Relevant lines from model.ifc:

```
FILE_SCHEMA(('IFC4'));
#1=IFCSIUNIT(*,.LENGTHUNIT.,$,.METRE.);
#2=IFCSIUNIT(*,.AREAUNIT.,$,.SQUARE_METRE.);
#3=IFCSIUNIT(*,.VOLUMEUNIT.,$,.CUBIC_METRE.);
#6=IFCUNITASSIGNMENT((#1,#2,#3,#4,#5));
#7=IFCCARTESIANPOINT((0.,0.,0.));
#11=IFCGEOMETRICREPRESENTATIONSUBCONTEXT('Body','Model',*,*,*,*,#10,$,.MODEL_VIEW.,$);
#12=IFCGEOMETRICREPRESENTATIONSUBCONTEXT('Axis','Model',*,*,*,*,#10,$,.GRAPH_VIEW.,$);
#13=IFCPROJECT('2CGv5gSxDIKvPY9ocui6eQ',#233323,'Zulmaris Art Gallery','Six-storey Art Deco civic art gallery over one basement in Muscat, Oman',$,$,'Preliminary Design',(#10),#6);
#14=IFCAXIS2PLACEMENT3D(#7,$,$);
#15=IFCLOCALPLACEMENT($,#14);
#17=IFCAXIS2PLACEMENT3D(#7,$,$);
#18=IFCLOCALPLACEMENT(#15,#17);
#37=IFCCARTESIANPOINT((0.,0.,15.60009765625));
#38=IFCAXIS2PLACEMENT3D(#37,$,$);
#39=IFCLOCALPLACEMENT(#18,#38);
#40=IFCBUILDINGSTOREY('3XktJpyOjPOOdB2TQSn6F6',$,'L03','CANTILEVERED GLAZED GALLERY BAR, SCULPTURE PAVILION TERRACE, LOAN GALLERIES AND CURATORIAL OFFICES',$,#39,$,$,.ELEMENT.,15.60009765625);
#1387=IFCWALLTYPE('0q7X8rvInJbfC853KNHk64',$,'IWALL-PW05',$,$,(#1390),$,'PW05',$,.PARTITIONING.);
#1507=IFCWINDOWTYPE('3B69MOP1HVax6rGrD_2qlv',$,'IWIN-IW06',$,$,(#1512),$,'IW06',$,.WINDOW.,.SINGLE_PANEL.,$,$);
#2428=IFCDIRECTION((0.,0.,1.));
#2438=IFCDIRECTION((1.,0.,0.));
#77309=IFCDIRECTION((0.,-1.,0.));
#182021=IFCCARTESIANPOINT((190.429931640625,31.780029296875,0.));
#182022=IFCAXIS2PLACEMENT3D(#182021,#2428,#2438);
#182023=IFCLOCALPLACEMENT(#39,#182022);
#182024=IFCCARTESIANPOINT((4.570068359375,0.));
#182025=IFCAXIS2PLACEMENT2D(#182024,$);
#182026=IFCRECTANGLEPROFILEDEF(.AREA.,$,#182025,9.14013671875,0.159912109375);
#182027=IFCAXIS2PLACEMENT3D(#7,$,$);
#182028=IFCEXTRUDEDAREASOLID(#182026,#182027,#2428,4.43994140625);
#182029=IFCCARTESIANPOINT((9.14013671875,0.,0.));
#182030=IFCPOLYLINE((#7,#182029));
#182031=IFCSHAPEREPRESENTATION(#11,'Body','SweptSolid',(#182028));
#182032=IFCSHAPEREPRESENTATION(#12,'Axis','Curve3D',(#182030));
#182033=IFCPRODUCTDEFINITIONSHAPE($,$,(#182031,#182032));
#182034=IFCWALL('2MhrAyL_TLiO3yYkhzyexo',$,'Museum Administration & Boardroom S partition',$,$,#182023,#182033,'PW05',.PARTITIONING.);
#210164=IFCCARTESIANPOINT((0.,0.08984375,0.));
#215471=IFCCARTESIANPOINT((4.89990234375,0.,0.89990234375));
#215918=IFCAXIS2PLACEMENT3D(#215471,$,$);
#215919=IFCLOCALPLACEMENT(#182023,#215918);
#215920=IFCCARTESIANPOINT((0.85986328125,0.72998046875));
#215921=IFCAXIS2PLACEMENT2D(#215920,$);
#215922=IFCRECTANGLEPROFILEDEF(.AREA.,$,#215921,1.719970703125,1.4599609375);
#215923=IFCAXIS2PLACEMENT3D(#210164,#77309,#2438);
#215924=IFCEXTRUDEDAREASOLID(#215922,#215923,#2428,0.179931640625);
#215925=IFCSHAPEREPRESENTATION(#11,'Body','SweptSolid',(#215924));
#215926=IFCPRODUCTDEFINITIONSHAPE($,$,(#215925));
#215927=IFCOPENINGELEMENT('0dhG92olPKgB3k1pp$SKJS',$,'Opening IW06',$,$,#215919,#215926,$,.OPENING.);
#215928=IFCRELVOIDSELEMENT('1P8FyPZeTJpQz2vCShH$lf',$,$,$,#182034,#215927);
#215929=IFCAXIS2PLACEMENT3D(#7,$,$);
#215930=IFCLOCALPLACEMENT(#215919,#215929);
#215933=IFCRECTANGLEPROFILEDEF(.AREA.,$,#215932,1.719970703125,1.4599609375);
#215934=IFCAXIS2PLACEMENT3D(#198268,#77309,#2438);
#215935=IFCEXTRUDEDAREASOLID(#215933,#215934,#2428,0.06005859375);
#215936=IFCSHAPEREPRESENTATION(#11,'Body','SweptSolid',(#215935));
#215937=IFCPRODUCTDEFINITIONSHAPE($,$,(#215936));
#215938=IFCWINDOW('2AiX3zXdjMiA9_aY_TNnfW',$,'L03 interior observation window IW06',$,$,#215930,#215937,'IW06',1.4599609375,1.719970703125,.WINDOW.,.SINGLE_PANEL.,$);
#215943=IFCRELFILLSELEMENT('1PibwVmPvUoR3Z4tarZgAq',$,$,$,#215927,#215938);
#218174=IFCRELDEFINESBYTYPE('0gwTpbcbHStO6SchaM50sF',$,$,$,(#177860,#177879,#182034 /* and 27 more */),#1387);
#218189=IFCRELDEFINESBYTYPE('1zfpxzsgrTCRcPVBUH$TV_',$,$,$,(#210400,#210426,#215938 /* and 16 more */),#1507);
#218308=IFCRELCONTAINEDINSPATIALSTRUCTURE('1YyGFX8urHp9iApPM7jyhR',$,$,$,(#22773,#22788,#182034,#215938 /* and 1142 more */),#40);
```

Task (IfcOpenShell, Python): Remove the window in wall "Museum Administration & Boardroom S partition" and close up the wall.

```python
import ifcopenshell
import ifcopenshell.api.feature
import ifcopenshell.api.root
import ifcopenshell.geom
import ifcopenshell.util.shape

model = ifcopenshell.open("model.ifc")
settings = ifcopenshell.geom.settings()


def volume(element):
    """Net volume in cubic metres, openings subtracted."""
    shape = ifcopenshell.geom.create_shape(settings, element)
    return ifcopenshell.util.shape.get_volume(shape.geometry)


window = model.by_id(215938)
opening = window.FillsVoids[0].RelatingOpeningElement
wall = opening.VoidsElements[0].RelatingBuildingElement
before = volume(wall)

ifcopenshell.api.root.remove_product(model, product=window)
ifcopenshell.api.feature.remove_feature(model, feature=opening)

after = volume(wall)

print(f"wall volume {before:.3f} -> {after:.3f} m3")

model.write("model_edited.ifc")
```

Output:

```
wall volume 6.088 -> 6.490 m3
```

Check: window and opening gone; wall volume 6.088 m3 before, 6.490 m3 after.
